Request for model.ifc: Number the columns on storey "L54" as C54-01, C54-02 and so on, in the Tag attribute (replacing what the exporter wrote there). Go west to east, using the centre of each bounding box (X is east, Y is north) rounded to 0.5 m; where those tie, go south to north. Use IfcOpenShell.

First a look at what the model holds.

```python
import ifcopenshell
import ifcopenshell.util.element
import ifcopenshell.util.placement

model = ifcopenshell.open("model.ifc")
print(model.schema)
storey = next(s for s in model.by_type("IfcBuildingStorey") if s.Name == "L54")
columns = [e for e in ifcopenshell.util.element.get_decomposition(storey) if e.is_a("IfcColumn")]
for e in sorted(columns, key=lambda e: e.id()):
    origin = ifcopenshell.util.placement.get_local_placement(e.ObjectPlacement)[:3, 3]
    print(e.id(), e.Tag, e.Name, origin.round(2) + 0.0, sep=" | ")
```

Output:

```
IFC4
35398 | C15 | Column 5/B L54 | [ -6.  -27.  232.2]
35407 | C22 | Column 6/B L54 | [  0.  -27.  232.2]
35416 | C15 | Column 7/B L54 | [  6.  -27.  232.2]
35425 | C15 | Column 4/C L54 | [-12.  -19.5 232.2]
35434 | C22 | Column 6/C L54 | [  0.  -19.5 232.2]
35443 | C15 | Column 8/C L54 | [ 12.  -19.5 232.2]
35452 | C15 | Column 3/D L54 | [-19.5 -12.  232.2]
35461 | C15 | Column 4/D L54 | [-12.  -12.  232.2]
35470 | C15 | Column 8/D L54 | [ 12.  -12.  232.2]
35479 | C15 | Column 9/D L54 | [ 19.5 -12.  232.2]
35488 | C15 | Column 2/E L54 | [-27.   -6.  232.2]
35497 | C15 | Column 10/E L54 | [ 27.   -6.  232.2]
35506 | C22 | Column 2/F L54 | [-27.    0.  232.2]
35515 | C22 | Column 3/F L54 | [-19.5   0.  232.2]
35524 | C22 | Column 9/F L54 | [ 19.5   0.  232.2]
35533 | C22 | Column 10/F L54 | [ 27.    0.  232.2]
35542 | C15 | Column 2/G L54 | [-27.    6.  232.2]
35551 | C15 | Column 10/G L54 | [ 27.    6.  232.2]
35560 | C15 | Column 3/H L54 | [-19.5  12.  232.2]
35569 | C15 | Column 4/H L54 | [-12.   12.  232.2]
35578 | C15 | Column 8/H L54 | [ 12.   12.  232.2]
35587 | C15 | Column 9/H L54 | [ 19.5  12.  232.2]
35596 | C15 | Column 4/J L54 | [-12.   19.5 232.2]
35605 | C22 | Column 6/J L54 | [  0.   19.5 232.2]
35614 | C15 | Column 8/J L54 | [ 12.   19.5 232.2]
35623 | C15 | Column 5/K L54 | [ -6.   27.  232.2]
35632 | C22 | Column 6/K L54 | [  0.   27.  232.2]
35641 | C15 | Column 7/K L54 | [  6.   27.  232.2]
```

```python
import ifcopenshell
import ifcopenshell.geom
import ifcopenshell.util.element
import ifcopenshell.util.shape

model = ifcopenshell.open("model.ifc")
settings = ifcopenshell.geom.settings()
settings.set("use-world-coords", True)


def centre(element):
    shape = ifcopenshell.geom.create_shape(settings, element)
    return ifcopenshell.util.shape.get_bbox_centroid(shape.geometry)


storey = next(s for s in model.by_type("IfcBuildingStorey") if s.Name == "L54")
columns = [e for e in ifcopenshell.util.element.get_decomposition(storey) if e.is_a("IfcColumn")]

# Insertion points can sit at a corner or the storey origin, so sort by the geometry (in metres).
centres = {e: centre(e) for e in columns}
columns.sort(key=lambda e: (round(centres[e][0] / 0.5), centres[e][1]))

for i, e in enumerate(columns, start=1):
    number = f"C54-{i:02d}"
    e.Tag = number
    print(e.id(), number)

model.write("model_edited.ifc")
```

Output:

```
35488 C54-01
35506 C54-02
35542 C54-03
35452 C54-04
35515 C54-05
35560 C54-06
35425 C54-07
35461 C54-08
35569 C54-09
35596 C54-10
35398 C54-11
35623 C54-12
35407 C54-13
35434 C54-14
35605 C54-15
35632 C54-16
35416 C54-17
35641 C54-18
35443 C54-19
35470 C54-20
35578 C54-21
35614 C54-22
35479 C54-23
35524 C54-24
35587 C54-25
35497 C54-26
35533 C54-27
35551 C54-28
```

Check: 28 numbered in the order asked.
